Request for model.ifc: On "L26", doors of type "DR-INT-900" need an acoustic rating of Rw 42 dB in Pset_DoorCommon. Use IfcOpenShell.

First a look at what the model holds.

```python
import ifcopenshell
import ifcopenshell.util.element

model = ifcopenshell.open("model.ifc")
print(model.schema)
storey = next(s for s in model.by_type("IfcBuildingStorey") if s.Name == "L26")
doors = [e for e in ifcopenshell.util.element.get_decomposition(storey) if e.is_a("IfcDoor")]
seen = {}
for e in doors:
    element_type = ifcopenshell.util.element.get_type(e)
    key = (element_type.Name if element_type != e and element_type else None, ifcopenshell.util.element.get_pset(e, "Pset_DoorCommon", "AcousticRating"))
    seen[key] = seen.get(key, 0) + 1
for (name, value), count in sorted(seen.items(), key=str):
    print(count, "x", name, "|", value)
```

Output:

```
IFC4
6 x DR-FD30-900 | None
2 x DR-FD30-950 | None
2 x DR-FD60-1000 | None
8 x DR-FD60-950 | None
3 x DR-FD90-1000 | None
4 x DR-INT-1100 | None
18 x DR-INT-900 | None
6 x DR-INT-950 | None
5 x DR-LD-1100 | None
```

```python
import ifcopenshell
import ifcopenshell.api.pset
import ifcopenshell.util.element

model = ifcopenshell.open("model.ifc")

storey = next(s for s in model.by_type("IfcBuildingStorey") if s.Name == "L26")
doors = [e for e in ifcopenshell.util.element.get_decomposition(storey) if e.is_a("IfcDoor")]

count = 0
for e in doors:
    element_type = ifcopenshell.util.element.get_type(e)
    if element_type in (None, e) or element_type.Name != "DR-INT-900":
        continue
    found = ifcopenshell.util.element.get_pset(e, "Pset_DoorCommon", should_inherit=False)
    if found:
        pset = model.by_id(found["id"])
        if len(ifcopenshell.util.element.get_elements_by_pset(pset)) > 1:
            pset = ifcopenshell.api.pset.unshare_pset(model, products=[e], pset=pset)[0]
    else:
        pset = ifcopenshell.api.pset.add_pset(model, product=e, name="Pset_DoorCommon")
    ifcopenshell.api.pset.edit_pset(model, pset=pset, properties={"AcousticRating": "Rw 42 dB"})
    count += 1

print(count, "doors updated")

model.write("model-out.ifc")
```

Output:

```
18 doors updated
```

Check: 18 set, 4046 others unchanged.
